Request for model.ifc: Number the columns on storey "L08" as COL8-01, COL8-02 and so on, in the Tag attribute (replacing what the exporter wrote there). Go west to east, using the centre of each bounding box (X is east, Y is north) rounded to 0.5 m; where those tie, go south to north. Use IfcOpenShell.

First a look at what the model holds.

```python
import ifcopenshell
import ifcopenshell.util.element
import ifcopenshell.util.placement

model = ifcopenshell.open("model.ifc")
print(model.schema)
storey = next(s for s in model.by_type("IfcBuildingStorey") if s.Name == "L08")
columns = [e for e in ifcopenshell.util.element.get_decomposition(storey) if e.is_a("IfcColumn")]
for e in sorted(columns, key=lambda e: e.id()):
    origin = ifcopenshell.util.placement.get_local_placement(e.ObjectPlacement)[:3, 3]
    print(e.id(), e.Tag, e.Name, origin.round(2) + 0.0, sep=" | ")
```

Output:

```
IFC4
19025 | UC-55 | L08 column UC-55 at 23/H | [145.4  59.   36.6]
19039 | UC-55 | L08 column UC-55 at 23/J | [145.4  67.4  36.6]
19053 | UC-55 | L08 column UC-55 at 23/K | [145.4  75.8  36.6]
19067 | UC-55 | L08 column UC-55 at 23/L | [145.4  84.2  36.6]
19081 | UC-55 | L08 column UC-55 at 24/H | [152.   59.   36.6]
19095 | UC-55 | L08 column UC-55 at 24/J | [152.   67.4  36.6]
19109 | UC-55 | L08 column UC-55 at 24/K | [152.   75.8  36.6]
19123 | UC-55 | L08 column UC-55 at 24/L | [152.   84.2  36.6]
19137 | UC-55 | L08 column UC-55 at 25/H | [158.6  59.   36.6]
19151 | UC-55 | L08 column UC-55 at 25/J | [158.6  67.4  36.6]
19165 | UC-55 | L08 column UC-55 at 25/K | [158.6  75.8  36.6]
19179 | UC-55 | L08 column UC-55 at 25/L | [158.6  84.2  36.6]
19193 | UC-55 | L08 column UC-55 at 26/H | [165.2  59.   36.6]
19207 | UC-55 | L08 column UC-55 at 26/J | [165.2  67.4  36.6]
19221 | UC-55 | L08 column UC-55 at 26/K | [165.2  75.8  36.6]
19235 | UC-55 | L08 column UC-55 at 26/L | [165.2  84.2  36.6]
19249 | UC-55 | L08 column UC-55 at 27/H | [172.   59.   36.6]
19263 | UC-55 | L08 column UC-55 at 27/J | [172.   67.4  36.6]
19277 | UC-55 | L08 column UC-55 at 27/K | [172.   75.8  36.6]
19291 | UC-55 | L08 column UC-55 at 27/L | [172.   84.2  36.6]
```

```python
import ifcopenshell
import ifcopenshell.geom
import ifcopenshell.util.element
import ifcopenshell.util.shape

model = ifcopenshell.open("model.ifc")
settings = ifcopenshell.geom.settings()
settings.set("use-world-coords", True)


def centre(element):
    shape = ifcopenshell.geom.create_shape(settings, element)
    return ifcopenshell.util.shape.get_bbox_centroid(shape.geometry)


storey = next(s for s in model.by_type("IfcBuildingStorey") if s.Name == "L08")
columns = [e for e in ifcopenshell.util.element.get_decomposition(storey) if e.is_a("IfcColumn")]

# Insertion points can sit at a corner or the storey origin, so sort by the geometry (in metres).
centres = {e: centre(e) for e in columns}
columns.sort(key=lambda e: (round(centres[e][0] / 0.5), centres[e][1]))

for i, e in enumerate(columns, start=1):
    number = f"COL8-{i:02d}"
    e.Tag = number
    print(e.id(), number)

model.write("model_updated.ifc")
```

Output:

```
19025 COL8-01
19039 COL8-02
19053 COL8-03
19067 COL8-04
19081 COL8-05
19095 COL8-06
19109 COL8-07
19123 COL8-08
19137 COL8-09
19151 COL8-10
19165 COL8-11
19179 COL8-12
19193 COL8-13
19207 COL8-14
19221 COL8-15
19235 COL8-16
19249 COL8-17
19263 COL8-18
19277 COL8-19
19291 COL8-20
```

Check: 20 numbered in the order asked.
